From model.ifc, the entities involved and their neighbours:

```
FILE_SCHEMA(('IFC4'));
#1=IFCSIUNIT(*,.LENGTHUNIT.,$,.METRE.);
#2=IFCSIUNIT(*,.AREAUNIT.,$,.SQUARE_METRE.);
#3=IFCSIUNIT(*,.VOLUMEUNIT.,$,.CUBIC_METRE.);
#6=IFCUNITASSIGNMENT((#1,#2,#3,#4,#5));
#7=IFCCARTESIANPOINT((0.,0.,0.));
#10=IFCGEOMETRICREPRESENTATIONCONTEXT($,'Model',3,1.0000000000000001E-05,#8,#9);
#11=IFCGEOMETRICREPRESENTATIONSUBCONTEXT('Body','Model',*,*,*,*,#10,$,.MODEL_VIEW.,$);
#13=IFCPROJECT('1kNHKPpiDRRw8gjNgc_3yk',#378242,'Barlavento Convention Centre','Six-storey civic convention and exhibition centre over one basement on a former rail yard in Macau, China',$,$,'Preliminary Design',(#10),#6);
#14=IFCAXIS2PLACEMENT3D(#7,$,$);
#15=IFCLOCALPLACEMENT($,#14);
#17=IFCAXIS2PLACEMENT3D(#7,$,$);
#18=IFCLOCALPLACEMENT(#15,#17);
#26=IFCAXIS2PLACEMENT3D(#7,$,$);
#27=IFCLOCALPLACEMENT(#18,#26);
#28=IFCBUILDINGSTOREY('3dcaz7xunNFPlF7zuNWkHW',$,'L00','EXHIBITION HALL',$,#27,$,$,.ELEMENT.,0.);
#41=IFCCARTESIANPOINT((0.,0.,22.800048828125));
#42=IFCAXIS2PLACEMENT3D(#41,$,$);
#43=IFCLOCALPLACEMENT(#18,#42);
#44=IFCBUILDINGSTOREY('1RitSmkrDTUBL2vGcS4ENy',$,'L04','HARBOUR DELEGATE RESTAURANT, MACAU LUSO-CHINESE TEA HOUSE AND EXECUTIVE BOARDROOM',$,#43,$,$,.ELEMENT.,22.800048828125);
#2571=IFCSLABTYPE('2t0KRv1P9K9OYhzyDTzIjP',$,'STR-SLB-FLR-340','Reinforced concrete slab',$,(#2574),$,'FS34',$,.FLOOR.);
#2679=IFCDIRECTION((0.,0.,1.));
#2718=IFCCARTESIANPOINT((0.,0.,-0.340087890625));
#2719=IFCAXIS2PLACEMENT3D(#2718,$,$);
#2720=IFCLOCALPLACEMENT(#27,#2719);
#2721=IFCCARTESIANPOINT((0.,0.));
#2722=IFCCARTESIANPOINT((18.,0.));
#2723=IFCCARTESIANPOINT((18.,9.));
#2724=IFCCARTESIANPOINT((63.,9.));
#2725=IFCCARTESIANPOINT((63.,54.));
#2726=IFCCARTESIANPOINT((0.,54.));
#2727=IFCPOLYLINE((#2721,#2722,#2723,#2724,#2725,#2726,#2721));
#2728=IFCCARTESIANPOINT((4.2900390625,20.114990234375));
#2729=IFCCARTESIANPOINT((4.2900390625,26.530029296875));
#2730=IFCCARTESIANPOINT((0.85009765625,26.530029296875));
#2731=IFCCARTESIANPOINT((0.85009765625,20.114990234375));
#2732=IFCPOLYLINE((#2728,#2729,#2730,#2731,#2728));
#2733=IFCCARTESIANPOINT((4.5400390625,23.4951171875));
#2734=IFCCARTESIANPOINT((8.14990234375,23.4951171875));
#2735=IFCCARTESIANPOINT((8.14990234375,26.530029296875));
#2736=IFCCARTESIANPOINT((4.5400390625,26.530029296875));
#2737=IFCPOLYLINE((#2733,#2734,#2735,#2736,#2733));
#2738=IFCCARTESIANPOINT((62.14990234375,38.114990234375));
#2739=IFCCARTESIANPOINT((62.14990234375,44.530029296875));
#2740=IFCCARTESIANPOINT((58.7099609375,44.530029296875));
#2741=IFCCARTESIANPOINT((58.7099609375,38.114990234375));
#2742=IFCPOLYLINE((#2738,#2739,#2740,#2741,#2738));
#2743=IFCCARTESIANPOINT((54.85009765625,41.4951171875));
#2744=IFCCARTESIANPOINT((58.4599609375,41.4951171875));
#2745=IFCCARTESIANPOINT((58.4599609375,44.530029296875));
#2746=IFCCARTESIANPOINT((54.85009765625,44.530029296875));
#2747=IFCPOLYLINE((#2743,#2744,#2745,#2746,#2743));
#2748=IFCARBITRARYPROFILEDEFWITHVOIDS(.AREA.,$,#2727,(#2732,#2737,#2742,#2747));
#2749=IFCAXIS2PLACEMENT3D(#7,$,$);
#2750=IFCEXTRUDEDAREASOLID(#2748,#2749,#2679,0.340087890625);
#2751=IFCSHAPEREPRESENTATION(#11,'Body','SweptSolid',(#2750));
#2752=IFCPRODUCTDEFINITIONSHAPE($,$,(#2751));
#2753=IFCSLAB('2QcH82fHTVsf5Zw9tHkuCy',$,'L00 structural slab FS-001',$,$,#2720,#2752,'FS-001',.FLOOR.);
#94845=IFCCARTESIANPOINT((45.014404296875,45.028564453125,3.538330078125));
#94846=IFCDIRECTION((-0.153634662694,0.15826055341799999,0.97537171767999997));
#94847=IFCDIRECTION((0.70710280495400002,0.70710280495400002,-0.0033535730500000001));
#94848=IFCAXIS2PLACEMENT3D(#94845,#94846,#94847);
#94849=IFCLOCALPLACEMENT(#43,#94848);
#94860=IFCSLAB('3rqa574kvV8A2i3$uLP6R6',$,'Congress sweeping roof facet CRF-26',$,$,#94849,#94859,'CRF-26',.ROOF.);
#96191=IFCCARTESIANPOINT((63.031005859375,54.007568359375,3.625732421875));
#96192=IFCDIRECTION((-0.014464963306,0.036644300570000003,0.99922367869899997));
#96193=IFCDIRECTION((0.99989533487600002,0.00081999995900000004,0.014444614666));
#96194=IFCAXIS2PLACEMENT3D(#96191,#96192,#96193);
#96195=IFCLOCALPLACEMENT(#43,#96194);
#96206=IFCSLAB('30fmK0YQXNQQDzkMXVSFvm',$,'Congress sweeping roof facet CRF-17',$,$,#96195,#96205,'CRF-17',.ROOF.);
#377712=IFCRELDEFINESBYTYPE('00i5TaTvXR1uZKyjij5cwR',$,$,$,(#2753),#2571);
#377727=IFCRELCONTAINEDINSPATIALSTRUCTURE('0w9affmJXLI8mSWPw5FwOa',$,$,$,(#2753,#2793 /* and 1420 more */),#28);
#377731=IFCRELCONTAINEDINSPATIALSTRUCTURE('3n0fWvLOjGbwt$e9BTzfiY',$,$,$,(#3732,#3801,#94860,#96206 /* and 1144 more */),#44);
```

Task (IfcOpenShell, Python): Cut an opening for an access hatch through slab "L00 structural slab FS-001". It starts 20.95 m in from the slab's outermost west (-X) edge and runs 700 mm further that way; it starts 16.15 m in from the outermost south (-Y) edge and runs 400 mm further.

```python
import numpy as np
import ifcopenshell
import ifcopenshell.api.feature
import ifcopenshell.api.geometry
import ifcopenshell.api.root
import ifcopenshell.geom
import ifcopenshell.util.placement
import ifcopenshell.util.representation
import ifcopenshell.util.shape
import ifcopenshell.util.unit

model = ifcopenshell.open("model.ifc")
unit_scale = ifcopenshell.util.unit.calculate_unit_scale(model)
settings = ifcopenshell.geom.settings()


def volume(element):
    """Net volume in cubic metres, openings subtracted."""
    shape = ifcopenshell.geom.create_shape(settings, element)
    return ifcopenshell.util.shape.get_volume(shape.geometry)


slab = model.by_guid("2QcH82fHTVsf5Zw9tHkuCy")
before = volume(slab)

# Extent in the slab's own axes, in metres. The edges named are its -X and -Y sides.
slab_shape = ifcopenshell.geom.create_shape(settings, slab)
vertices = ifcopenshell.util.shape.get_vertices(slab_shape.geometry)
x_min, y_min, bottom = vertices.min(axis=0)
top = vertices[:, 2].max()

opening = ifcopenshell.api.root.create_entity(model, ifc_class="IfcOpeningElement", name="Access hatch opening", predefined_type="OPENING")
context = ifcopenshell.util.representation.get_context(model, "Model", "Body", "MODEL_VIEW")
width, depth = 0.7, 0.4
outline = [(0.0, 0.0), (width, 0.0), (width, depth), (0.0, depth), (0.0, 0.0)]
# Overshoot both faces by 50 mm so the cut is clean.
shape = ifcopenshell.api.geometry.add_slab_representation(
    model, context=context, depth=top - bottom + 0.1, polyline=outline
)
ifcopenshell.api.geometry.assign_representation(model, product=opening, representation=shape)

matrix = ifcopenshell.util.placement.get_local_placement(slab.ObjectPlacement)
matrix[:, 3] = matrix @ np.append(np.array([x_min + 20.95, y_min + 16.15, bottom - 0.05]) / unit_scale, 1.0)
ifcopenshell.api.geometry.edit_object_placement(model, product=opening, matrix=matrix, is_si=False)
ifcopenshell.api.feature.add_feature(model, feature=opening, element=slab)

after = volume(slab)

print(f"slab volume {before:.3f} -> {after:.3f} m3")

model.write("model-out.ifc")
```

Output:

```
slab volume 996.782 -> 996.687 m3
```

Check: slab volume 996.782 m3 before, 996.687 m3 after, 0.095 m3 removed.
